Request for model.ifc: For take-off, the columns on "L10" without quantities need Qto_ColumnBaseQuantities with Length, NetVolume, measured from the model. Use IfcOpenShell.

First a look at what the model holds.

```python
import ifcopenshell
import ifcopenshell.util.element
import ifcopenshell.util.unit

model = ifcopenshell.open("model.ifc")
print(model.schema)
for unit_type in ("LENGTHUNIT", "AREAUNIT", "VOLUMEUNIT"):
    print(unit_type, ifcopenshell.util.unit.calculate_unit_scale(model, unit_type))
storey = next(s for s in model.by_type("IfcBuildingStorey") if s.Name == "L10")
columns = [e for e in ifcopenshell.util.element.get_decomposition(storey) if e.is_a("IfcColumn")]
for e in sorted(columns, key=lambda e: e.id()):
    print(e.id(), e.is_a(), e.Name, list(ifcopenshell.util.element.get_psets(e, qtos_only=True)), sep=" | ")
```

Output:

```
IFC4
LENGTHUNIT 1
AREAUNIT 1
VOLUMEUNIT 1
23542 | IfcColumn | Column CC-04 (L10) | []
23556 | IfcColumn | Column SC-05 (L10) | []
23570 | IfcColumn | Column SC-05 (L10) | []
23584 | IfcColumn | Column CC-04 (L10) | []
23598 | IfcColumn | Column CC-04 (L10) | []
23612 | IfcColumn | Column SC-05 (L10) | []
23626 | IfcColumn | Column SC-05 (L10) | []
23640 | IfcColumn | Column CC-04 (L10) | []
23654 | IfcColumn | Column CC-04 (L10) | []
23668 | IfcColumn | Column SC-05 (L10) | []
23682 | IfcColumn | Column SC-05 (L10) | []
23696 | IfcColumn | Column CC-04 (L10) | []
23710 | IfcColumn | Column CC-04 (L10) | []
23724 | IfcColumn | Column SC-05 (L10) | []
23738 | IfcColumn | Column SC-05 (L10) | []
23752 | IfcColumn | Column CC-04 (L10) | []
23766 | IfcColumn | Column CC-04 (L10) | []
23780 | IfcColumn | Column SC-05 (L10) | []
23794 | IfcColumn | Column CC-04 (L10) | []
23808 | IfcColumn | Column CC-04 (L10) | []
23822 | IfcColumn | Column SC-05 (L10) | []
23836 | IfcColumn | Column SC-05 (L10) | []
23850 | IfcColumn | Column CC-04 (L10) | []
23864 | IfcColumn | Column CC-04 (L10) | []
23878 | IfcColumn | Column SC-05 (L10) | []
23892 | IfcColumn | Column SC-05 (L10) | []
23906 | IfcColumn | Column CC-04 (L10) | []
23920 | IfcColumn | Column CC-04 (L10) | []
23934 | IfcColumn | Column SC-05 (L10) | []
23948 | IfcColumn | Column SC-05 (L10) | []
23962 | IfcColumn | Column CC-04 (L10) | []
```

```python
import ifcopenshell
import ifcopenshell.api.pset
import ifcopenshell.geom
import ifcopenshell.util.element
import ifcopenshell.util.shape
import ifcopenshell.util.unit

model = ifcopenshell.open("model.ifc")
unit_scale = ifcopenshell.util.unit.calculate_unit_scale(model)
volume_scale = ifcopenshell.util.unit.calculate_unit_scale(model, "VOLUMEUNIT")
settings = ifcopenshell.geom.settings()

storey = next(s for s in model.by_type("IfcBuildingStorey") if s.Name == "L10")
columns = [e for e in ifcopenshell.util.element.get_decomposition(storey) if e.is_a("IfcColumn")]

for e in sorted(columns, key=lambda e: e.id()):
    if ifcopenshell.util.element.get_psets(e, qtos_only=True, should_inherit=False):
        continue
    # Geometry comes back in metres, in the element's own axes.
    shape = ifcopenshell.geom.create_shape(settings, e)
    values = {
        "Length": ifcopenshell.util.shape.get_z(shape.geometry) / unit_scale,
        "NetVolume": ifcopenshell.util.shape.get_volume(shape.geometry) / volume_scale,
    }
    qto = ifcopenshell.api.pset.add_qto(model, product=e, name="Qto_ColumnBaseQuantities")
    ifcopenshell.api.pset.edit_qto(model, qto=qto, properties=values)
    print(e.id(), {k: round(v, 3) for k, v in values.items()})

model.write("model_v2.ifc")
```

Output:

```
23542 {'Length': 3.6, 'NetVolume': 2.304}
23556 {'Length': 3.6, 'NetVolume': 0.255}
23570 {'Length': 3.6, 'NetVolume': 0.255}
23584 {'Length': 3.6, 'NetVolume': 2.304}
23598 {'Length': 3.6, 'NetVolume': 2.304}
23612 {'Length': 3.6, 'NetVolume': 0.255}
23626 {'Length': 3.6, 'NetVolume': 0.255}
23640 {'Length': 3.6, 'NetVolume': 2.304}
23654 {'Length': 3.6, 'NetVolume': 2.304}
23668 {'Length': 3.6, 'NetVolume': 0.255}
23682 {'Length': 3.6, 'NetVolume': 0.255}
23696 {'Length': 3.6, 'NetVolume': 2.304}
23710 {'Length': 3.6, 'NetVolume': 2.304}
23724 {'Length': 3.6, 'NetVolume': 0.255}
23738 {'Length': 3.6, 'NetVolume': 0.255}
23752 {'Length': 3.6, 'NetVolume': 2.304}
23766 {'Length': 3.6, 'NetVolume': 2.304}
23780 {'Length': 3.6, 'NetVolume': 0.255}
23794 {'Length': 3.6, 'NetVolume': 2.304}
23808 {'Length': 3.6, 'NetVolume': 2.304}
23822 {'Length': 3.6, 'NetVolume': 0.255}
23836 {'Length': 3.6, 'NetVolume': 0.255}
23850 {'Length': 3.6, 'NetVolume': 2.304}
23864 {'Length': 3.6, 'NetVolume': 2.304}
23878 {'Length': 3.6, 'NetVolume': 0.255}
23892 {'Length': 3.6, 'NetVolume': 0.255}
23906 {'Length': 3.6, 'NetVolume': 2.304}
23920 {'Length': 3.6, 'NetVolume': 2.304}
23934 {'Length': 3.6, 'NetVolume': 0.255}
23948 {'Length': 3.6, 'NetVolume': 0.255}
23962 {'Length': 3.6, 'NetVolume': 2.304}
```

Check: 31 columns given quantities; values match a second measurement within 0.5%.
